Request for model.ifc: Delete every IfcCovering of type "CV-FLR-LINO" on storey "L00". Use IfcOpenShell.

First a look at what the model holds.

```python
import ifcopenshell
import ifcopenshell.util.element

model = ifcopenshell.open("model.ifc")
print(model.schema)
storey = next(s for s in model.by_type("IfcBuildingStorey") if s.Name == "L00")
coverings = [e for e in ifcopenshell.util.element.get_decomposition(storey) if e.is_a("IfcCovering")]
seen = {}
for e in coverings:
    element_type = ifcopenshell.util.element.get_type(e)
    name = element_type.Name if element_type not in (None, e) else None
    seen[name] = seen.get(name, 0) + 1
for name, count in sorted(seen.items(), key=str):
    print(count, "x", name)
```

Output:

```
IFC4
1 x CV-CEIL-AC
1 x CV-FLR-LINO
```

```python
import ifcopenshell
import ifcopenshell.api.root
import ifcopenshell.util.element

model = ifcopenshell.open("model.ifc")

storey = next(s for s in model.by_type("IfcBuildingStorey") if s.Name == "L00")
coverings = [e for e in ifcopenshell.util.element.get_decomposition(storey) if e.is_a("IfcCovering")]
targets = [e for e in coverings if (t := ifcopenshell.util.element.get_type(e)) not in (None, e) and t.Name == "CV-FLR-LINO"]

for e in targets:
    ifcopenshell.api.root.remove_product(model, product=e)
print(len(targets), "removed")

model.write("model_updated.ifc")
```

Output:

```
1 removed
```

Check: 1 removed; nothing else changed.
